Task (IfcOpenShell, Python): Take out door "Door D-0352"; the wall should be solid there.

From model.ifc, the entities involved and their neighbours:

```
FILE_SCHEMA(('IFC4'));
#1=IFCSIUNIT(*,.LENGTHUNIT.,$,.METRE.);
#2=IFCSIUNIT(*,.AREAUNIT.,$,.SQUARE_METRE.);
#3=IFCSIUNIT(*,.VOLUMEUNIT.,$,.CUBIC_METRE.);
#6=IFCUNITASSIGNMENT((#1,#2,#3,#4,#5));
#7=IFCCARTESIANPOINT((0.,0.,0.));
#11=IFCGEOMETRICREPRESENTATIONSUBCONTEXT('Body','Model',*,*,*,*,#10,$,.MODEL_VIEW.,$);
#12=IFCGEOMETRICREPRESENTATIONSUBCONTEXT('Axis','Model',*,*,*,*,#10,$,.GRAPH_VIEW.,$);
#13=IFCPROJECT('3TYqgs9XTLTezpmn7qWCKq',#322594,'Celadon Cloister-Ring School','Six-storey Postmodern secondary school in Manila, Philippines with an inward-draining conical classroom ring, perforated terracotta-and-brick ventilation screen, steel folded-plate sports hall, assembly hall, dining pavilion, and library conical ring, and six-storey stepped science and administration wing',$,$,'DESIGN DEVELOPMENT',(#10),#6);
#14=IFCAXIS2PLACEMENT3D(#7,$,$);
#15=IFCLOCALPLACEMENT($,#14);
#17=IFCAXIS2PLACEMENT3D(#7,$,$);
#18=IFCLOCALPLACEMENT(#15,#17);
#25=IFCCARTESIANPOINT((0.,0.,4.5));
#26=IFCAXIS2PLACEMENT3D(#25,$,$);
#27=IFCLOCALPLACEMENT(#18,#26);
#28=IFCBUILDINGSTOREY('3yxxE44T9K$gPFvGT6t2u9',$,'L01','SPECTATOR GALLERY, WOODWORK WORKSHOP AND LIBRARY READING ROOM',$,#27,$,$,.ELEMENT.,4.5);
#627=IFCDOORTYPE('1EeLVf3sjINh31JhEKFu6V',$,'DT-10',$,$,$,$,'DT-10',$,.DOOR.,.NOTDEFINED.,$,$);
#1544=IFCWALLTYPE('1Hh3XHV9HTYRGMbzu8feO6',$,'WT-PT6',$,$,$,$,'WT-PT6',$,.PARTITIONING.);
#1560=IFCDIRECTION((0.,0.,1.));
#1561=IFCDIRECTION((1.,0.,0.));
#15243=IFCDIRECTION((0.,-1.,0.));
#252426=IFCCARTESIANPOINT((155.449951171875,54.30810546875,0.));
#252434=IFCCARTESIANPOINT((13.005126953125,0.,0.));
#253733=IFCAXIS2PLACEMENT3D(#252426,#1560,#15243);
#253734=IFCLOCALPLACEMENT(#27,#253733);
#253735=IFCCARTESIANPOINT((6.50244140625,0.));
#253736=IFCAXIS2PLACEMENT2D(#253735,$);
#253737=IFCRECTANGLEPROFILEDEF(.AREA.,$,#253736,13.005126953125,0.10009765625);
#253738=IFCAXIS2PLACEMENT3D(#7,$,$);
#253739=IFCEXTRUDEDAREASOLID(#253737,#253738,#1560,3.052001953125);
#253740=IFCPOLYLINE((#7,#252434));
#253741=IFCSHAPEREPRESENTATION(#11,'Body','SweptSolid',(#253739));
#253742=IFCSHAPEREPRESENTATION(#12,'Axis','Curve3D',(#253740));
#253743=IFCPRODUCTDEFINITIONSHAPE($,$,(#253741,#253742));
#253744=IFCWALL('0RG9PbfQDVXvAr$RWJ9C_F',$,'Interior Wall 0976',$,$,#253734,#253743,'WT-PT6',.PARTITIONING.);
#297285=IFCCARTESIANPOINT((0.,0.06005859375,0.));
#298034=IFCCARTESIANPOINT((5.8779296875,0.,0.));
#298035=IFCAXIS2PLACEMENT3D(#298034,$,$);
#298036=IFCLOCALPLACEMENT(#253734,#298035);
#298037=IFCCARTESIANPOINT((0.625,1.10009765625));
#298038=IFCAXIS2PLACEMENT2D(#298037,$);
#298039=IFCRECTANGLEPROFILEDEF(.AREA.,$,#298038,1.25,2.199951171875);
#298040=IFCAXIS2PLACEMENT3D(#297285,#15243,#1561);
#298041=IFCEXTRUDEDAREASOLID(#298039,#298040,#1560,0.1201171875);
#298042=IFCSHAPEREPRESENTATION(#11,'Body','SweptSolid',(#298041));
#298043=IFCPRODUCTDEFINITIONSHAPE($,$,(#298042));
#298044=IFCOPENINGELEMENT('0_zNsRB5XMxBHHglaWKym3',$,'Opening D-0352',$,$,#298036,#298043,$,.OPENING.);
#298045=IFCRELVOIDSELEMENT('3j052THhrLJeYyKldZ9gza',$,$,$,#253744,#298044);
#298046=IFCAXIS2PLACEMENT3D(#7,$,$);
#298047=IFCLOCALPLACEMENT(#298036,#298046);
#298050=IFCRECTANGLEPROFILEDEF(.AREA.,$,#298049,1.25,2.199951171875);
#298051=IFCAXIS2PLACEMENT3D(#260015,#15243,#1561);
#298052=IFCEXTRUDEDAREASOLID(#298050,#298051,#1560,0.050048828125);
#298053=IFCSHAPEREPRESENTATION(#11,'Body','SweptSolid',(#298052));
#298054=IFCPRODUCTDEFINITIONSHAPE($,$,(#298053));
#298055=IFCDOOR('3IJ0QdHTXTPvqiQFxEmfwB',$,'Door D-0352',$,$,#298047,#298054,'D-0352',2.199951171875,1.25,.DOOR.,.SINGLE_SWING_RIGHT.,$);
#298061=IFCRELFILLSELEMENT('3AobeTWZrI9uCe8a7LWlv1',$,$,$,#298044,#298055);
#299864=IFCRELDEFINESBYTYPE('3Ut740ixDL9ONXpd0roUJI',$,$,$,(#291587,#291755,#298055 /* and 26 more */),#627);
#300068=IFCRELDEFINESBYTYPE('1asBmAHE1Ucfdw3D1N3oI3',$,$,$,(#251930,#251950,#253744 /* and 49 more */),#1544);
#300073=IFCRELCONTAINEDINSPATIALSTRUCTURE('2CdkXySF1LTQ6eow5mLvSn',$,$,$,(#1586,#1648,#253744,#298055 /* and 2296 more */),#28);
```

```python
import ifcopenshell
import ifcopenshell.api.feature
import ifcopenshell.api.root
import ifcopenshell.geom
import ifcopenshell.util.shape

model = ifcopenshell.open("model.ifc")
settings = ifcopenshell.geom.settings()


def volume(element):
    """Net volume in cubic metres, openings subtracted."""
    shape = ifcopenshell.geom.create_shape(settings, element)
    return ifcopenshell.util.shape.get_volume(shape.geometry)


door = model.by_guid("3IJ0QdHTXTPvqiQFxEmfwB")
opening = door.FillsVoids[0].RelatingOpeningElement
wall = opening.VoidsElements[0].RelatingBuildingElement
before = volume(wall)

ifcopenshell.api.root.remove_product(model, product=door)
ifcopenshell.api.feature.remove_feature(model, feature=opening)

after = volume(wall)

print(f"wall volume {before:.3f} -> {after:.3f} m3")

model.write("model_updated.ifc")
```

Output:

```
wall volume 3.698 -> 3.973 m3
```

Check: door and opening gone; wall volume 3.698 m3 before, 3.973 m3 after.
